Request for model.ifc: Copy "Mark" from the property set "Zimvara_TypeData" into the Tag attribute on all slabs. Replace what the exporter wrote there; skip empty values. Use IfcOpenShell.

First a look at what the model holds.

```python
import ifcopenshell
import ifcopenshell.util.element

model = ifcopenshell.open("model.ifc")
print(model.schema)
slabs = model.by_type("IfcSlab")
print(len(slabs), "slabs")
for e in slabs[:8]:
    source = ifcopenshell.util.element.get_pset(e, "Zimvara_TypeData", "Mark")
    target = e.Tag
    print(e.id(), repr(source), repr(target), sep=" | ")
```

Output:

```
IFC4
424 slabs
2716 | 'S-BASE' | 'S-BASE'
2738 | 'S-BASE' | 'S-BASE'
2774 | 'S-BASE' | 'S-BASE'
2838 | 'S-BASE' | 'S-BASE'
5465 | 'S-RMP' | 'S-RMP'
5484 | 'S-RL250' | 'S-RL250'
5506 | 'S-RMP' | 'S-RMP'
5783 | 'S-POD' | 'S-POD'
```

```python
import ifcopenshell
import ifcopenshell.util.element

model = ifcopenshell.open("model.ifc")

count = 0
for e in model.by_type("IfcSlab"):
    value = ifcopenshell.util.element.get_pset(e, "Zimvara_TypeData", "Mark")
    current = e.Tag
    if not value or not value.strip() or current == value:
        continue
    e.Tag = value
    count += 1

print(count, "slabs updated")

model.write("model-out.ifc")
```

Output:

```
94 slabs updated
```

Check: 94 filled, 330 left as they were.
